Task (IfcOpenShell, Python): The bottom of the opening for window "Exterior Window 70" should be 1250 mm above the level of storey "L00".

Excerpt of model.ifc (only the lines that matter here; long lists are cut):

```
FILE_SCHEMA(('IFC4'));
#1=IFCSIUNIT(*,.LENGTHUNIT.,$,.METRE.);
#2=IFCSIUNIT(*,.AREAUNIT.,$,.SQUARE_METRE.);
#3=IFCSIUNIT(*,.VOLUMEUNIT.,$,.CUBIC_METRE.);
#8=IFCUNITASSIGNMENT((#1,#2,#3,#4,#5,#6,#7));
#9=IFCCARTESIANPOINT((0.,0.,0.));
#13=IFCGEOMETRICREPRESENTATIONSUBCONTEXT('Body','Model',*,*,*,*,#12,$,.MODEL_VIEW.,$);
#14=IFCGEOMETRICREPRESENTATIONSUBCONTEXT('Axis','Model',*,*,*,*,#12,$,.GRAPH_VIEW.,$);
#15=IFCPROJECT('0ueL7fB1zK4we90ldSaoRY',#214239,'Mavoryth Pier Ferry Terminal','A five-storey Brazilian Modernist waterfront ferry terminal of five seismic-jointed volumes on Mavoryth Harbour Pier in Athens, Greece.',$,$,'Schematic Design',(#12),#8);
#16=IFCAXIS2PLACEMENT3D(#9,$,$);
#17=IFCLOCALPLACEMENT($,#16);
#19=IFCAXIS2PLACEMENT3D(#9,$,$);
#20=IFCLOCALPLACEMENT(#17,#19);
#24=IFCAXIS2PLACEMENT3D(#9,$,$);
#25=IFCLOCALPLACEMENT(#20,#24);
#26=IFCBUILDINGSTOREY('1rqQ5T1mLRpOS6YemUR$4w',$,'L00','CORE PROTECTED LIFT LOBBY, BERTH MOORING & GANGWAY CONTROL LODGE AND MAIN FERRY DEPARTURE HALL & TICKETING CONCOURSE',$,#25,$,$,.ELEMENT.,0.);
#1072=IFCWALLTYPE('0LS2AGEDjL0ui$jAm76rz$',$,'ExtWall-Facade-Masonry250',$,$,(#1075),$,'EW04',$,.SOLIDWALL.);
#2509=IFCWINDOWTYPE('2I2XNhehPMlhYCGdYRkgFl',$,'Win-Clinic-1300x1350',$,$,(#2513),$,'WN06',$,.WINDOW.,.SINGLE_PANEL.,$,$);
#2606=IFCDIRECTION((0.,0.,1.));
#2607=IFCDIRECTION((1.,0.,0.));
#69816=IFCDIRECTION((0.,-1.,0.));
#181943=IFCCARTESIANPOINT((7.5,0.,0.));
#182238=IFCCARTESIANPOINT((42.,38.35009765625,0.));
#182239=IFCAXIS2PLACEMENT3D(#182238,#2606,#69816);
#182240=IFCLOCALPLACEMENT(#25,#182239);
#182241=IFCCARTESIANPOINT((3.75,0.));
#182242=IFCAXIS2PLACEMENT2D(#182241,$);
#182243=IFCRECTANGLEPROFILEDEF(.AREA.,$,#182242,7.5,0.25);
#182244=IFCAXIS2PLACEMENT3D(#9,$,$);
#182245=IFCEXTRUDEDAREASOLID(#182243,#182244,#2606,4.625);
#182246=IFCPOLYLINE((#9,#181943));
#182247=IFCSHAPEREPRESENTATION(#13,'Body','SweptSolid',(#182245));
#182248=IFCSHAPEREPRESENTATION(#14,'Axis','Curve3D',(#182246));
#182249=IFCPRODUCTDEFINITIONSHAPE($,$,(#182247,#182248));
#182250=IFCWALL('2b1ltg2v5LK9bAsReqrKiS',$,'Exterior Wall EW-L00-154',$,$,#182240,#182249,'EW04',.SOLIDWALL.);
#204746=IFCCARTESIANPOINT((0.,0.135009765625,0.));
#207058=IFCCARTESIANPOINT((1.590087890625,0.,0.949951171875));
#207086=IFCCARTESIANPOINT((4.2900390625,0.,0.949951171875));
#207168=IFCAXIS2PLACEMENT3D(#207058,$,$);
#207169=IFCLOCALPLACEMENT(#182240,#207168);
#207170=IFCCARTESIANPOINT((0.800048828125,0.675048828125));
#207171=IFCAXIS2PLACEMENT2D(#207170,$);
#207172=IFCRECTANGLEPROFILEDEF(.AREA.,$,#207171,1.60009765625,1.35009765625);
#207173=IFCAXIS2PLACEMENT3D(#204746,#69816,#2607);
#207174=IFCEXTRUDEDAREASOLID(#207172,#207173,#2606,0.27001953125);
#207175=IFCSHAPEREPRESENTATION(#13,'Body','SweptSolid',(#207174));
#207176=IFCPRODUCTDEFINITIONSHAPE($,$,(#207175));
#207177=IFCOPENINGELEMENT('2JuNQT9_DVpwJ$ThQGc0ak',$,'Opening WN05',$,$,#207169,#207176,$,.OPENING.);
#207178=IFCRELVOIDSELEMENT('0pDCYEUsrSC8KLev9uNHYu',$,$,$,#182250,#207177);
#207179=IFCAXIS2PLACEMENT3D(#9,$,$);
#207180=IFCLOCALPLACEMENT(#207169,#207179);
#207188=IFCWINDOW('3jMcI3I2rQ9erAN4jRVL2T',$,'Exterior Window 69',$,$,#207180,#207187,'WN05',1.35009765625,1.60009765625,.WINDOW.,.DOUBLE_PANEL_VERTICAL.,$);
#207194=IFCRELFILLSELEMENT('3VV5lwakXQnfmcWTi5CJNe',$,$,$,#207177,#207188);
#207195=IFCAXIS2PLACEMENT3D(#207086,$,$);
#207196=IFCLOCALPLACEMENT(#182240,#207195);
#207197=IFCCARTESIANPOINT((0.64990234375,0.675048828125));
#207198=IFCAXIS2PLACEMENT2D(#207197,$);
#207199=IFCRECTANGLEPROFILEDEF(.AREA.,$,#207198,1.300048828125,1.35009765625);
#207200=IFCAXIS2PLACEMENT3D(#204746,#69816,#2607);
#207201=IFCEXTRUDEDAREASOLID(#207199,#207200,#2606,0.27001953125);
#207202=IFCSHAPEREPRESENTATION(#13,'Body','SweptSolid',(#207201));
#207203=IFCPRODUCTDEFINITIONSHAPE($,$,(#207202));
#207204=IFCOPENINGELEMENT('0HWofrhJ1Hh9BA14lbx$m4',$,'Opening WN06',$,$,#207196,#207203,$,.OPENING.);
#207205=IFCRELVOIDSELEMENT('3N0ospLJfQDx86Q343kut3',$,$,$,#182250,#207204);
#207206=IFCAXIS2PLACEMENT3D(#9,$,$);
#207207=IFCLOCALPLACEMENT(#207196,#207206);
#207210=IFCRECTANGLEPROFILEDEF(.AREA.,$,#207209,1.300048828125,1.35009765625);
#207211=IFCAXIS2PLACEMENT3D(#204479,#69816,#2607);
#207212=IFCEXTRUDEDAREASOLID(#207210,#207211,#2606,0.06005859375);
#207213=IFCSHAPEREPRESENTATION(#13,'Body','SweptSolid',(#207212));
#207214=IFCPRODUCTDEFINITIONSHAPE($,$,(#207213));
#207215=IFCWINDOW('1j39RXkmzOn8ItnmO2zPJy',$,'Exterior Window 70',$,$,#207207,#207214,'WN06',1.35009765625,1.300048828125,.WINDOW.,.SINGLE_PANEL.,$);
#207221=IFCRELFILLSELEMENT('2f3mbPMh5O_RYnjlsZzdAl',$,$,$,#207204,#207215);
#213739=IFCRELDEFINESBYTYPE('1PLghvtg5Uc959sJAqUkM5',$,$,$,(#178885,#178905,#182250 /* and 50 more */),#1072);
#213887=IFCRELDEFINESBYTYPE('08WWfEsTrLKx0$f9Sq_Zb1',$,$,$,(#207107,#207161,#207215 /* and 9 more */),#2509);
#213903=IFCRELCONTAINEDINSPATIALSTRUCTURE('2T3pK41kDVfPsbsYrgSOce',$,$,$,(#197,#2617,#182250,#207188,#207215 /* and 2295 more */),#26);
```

```python
import numpy as np
import ifcopenshell
import ifcopenshell.api.geometry
import ifcopenshell.geom
import ifcopenshell.util.element
import ifcopenshell.util.placement
import ifcopenshell.util.shape
import ifcopenshell.util.unit

model = ifcopenshell.open("model.ifc")
unit_scale = ifcopenshell.util.unit.calculate_unit_scale(model)

window = model.by_guid("1j39RXkmzOn8ItnmO2zPJy")
opening = window.FillsVoids[0].RelatingOpeningElement
storey = ifcopenshell.util.element.get_container(window, ifc_class="IfcBuildingStorey")
level = ifcopenshell.util.placement.get_local_placement(storey.ObjectPlacement)[2, 3]

# The opening's origin need not be at the sill, so measure its lowest point.
shape = ifcopenshell.geom.create_shape(ifcopenshell.geom.settings(), opening)
bottom = ifcopenshell.util.shape.get_shape_bottom_elevation(shape, shape.geometry) / unit_scale
dz = level + 1.25 / unit_scale - bottom

shift = np.array([0.0, 0.0, dz])
# The window is placed relative to its opening, so it follows when the opening moves.
matrix = ifcopenshell.util.placement.get_local_placement(opening.ObjectPlacement)
matrix[:3, 3] += shift
ifcopenshell.api.geometry.edit_object_placement(
    model, product=opening, matrix=matrix, is_si=False, should_transform_children=True
)

print(f"moved by {dz * unit_scale:+.3f} m")

model.write("model_rev.ifc")
```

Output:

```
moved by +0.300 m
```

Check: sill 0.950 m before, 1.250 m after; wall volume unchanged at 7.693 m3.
